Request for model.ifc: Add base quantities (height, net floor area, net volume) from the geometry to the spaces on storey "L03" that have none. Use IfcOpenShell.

First a look at what the model holds.

```python
import ifcopenshell
import ifcopenshell.util.element
import ifcopenshell.util.unit

model = ifcopenshell.open("model.ifc")
print(model.schema)
for unit_type in ("LENGTHUNIT", "AREAUNIT", "VOLUMEUNIT"):
    print(unit_type, ifcopenshell.util.unit.calculate_unit_scale(model, unit_type))
storey = next(s for s in model.by_type("IfcBuildingStorey") if s.Name == "L03")
spaces = [e for e in ifcopenshell.util.element.get_decomposition(storey) if e.is_a("IfcSpace")]
for e in sorted(spaces, key=lambda e: e.id()):
    print(e.id(), e.is_a(), e.Name, list(ifcopenshell.util.element.get_psets(e, qtos_only=True)), sep=" | ")
```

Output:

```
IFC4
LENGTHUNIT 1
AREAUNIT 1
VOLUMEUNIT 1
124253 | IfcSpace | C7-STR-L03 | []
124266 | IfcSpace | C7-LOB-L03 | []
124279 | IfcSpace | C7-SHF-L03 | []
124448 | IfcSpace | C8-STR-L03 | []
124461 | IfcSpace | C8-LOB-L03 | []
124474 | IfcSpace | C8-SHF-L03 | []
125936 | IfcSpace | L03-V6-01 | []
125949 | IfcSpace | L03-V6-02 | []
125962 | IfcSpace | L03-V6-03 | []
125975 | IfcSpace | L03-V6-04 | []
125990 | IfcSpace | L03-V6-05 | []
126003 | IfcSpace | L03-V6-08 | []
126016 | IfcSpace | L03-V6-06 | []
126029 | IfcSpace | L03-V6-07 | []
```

```python
import ifcopenshell
import ifcopenshell.api.pset
import ifcopenshell.geom
import ifcopenshell.util.element
import ifcopenshell.util.shape
import ifcopenshell.util.unit

model = ifcopenshell.open("model.ifc")
unit_scale = ifcopenshell.util.unit.calculate_unit_scale(model)
area_scale = ifcopenshell.util.unit.calculate_unit_scale(model, "AREAUNIT")
volume_scale = ifcopenshell.util.unit.calculate_unit_scale(model, "VOLUMEUNIT")
settings = ifcopenshell.geom.settings()

storey = next(s for s in model.by_type("IfcBuildingStorey") if s.Name == "L03")
spaces = [e for e in ifcopenshell.util.element.get_decomposition(storey) if e.is_a("IfcSpace")]

for e in sorted(spaces, key=lambda e: e.id()):
    if ifcopenshell.util.element.get_psets(e, qtos_only=True, should_inherit=False):
        continue
    # Geometry comes back in metres, in the element's own axes.
    shape = ifcopenshell.geom.create_shape(settings, e)
    values = {
        "Height": ifcopenshell.util.shape.get_z(shape.geometry) / unit_scale,
        "NetFloorArea": ifcopenshell.util.shape.get_footprint_area(shape.geometry) / area_scale,
        "NetVolume": ifcopenshell.util.shape.get_volume(shape.geometry) / volume_scale,
    }
    qto = ifcopenshell.api.pset.add_qto(model, product=e, name="Qto_SpaceBaseQuantities")
    ifcopenshell.api.pset.edit_qto(model, qto=qto, properties=values)
    print(e.id(), {k: round(v, 3) for k, v in values.items()})

model.write("model_v2.ifc")
```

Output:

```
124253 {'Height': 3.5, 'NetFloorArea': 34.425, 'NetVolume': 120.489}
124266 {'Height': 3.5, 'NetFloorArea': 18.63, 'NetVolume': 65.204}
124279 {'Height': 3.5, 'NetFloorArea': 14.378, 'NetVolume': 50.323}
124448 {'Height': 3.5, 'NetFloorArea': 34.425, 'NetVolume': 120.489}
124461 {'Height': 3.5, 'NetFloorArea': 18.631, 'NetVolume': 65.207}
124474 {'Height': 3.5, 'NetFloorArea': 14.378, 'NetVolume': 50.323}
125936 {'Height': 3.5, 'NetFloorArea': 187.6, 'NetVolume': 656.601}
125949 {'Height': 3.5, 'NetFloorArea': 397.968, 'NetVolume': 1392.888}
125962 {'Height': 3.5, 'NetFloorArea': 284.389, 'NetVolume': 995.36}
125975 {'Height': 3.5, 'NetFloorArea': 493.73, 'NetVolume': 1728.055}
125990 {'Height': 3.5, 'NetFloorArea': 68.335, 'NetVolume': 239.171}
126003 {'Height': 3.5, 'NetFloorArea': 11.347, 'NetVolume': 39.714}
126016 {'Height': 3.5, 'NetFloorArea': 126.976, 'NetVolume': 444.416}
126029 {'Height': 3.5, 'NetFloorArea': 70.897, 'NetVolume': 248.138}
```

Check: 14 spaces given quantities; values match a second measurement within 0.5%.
